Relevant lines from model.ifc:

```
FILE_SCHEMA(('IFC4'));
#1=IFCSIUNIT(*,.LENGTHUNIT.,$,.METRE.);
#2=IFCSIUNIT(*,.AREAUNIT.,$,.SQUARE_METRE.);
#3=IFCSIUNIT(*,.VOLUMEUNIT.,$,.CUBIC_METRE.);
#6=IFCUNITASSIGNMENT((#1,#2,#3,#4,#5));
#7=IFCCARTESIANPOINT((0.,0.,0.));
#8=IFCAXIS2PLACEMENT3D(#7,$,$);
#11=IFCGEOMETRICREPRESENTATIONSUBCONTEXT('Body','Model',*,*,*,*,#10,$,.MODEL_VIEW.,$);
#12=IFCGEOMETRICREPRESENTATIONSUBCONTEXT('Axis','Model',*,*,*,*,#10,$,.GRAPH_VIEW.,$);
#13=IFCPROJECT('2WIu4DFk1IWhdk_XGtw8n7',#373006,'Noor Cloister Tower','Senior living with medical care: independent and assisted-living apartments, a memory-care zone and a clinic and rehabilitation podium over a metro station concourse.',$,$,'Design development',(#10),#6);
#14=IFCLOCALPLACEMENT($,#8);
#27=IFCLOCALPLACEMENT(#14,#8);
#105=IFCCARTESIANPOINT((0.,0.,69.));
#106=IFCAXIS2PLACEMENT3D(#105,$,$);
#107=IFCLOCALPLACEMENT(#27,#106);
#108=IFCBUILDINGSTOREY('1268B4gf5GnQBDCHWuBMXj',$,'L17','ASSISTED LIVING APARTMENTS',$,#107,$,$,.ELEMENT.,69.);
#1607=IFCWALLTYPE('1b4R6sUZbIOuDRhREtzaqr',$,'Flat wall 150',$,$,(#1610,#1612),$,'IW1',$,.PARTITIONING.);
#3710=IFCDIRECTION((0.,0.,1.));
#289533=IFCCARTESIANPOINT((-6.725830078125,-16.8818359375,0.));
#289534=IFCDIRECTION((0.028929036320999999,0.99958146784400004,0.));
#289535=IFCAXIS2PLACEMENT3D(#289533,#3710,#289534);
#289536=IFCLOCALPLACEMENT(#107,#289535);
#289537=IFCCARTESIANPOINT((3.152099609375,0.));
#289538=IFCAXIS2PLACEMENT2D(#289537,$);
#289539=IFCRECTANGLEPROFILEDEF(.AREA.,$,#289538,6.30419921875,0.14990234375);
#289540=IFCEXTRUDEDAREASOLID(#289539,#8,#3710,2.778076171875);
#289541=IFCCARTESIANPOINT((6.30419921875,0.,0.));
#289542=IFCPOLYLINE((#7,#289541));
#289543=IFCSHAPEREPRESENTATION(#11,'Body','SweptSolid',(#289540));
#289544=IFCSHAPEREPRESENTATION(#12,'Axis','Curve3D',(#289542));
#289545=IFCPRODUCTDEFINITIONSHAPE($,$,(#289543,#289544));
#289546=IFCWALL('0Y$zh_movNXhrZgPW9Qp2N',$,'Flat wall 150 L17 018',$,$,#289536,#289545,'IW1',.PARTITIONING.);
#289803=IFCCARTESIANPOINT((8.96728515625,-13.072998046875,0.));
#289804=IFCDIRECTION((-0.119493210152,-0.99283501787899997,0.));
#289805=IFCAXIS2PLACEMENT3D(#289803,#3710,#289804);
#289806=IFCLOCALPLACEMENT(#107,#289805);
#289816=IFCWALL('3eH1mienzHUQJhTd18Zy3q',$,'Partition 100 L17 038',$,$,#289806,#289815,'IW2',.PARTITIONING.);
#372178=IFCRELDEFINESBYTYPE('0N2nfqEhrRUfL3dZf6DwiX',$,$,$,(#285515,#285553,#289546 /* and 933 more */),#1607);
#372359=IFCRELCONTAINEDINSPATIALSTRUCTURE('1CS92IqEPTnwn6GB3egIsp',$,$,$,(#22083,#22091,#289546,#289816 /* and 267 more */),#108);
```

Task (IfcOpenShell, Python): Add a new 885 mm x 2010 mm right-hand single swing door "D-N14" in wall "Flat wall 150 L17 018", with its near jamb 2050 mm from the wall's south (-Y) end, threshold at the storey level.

```python
import numpy as np
import ifcopenshell
import ifcopenshell.api.feature
import ifcopenshell.api.geometry
import ifcopenshell.api.root
import ifcopenshell.api.spatial
import ifcopenshell.geom
import ifcopenshell.util.element
import ifcopenshell.util.placement
import ifcopenshell.util.representation
import ifcopenshell.util.shape
import ifcopenshell.util.unit

model = ifcopenshell.open("model.ifc")
unit_scale = ifcopenshell.util.unit.calculate_unit_scale(model)
settings = ifcopenshell.geom.settings()


def volume(element):
    """Net volume in cubic metres, openings subtracted."""
    shape = ifcopenshell.geom.create_shape(settings, element)
    return ifcopenshell.util.shape.get_volume(shape.geometry)


wall = model.by_id(289546)
storey = ifcopenshell.util.element.get_container(wall, ifc_class="IfcBuildingStorey")
context = ifcopenshell.util.representation.get_context(model, "Model", "Body", "MODEL_VIEW")
before = volume(wall)

width, height, from_end, sill = 0.885, 2.01, 2.05, 0.0  # metres

# The wall runs along its own X axis, and the end named is its -X end.
wall_shape = ifcopenshell.geom.create_shape(settings, wall)
x, y, z = ifcopenshell.util.shape.get_vertices(wall_shape.geometry).T
start = x.min() + from_end
face, thickness = float(y.min()), float(y.max() - y.min())
wall_matrix = ifcopenshell.util.placement.get_local_placement(wall.ObjectPlacement)
level = ifcopenshell.util.placement.get_local_placement(storey.ObjectPlacement)[2, 3]


def in_wall(x, y):
    """Placement at x, y metres in the wall's axes, at sill height."""
    matrix = wall_matrix.copy()
    matrix[:, 3] = wall_matrix @ np.array([x / unit_scale, y / unit_scale, 0.0, 1.0])
    matrix[2, 3] = level + sill / unit_scale
    return matrix


# Opening: a box that overshoots both wall faces by 50 mm.
opening = ifcopenshell.api.root.create_entity(model, ifc_class="IfcOpeningElement", predefined_type="OPENING")
box = ifcopenshell.api.geometry.add_wall_representation(
    model, context=context, length=width, height=height, thickness=thickness + 0.1
)
ifcopenshell.api.geometry.assign_representation(model, product=opening, representation=box)
ifcopenshell.api.geometry.edit_object_placement(model, product=opening, matrix=in_wall(start, face - 0.05), is_si=False)
ifcopenshell.api.feature.add_feature(model, feature=opening, element=wall)

door = ifcopenshell.api.root.create_entity(model, ifc_class="IfcDoor", name="D-N14", predefined_type="DOOR")
door.OverallWidth, door.OverallHeight = width / unit_scale, height / unit_scale
door.OperationType = "SINGLE_SWING_RIGHT"
body = ifcopenshell.api.geometry.add_door_representation(
    model,
    context=context,
    overall_width=door.OverallWidth,
    overall_height=door.OverallHeight,
    operation_type="SINGLE_SWING_RIGHT",
    lining_properties={"LiningDepth": thickness / unit_scale, "ThresholdDepth": thickness / unit_scale},
)
ifcopenshell.api.geometry.assign_representation(model, product=door, representation=body)
ifcopenshell.api.spatial.assign_container(model, products=[door], relating_structure=storey)
ifcopenshell.api.feature.add_filling(model, opening=opening, element=door)

# The lining spans the wall, so the door starts at the wall face.
ifcopenshell.api.geometry.edit_object_placement(model, product=door, matrix=in_wall(start, face), is_si=False)

after = volume(wall)

print(f"wall volume {before:.3f} -> {after:.3f} m3")

model.write("model_edited.ifc")
```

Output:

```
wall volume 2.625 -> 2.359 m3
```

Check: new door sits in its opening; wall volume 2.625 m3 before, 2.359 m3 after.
